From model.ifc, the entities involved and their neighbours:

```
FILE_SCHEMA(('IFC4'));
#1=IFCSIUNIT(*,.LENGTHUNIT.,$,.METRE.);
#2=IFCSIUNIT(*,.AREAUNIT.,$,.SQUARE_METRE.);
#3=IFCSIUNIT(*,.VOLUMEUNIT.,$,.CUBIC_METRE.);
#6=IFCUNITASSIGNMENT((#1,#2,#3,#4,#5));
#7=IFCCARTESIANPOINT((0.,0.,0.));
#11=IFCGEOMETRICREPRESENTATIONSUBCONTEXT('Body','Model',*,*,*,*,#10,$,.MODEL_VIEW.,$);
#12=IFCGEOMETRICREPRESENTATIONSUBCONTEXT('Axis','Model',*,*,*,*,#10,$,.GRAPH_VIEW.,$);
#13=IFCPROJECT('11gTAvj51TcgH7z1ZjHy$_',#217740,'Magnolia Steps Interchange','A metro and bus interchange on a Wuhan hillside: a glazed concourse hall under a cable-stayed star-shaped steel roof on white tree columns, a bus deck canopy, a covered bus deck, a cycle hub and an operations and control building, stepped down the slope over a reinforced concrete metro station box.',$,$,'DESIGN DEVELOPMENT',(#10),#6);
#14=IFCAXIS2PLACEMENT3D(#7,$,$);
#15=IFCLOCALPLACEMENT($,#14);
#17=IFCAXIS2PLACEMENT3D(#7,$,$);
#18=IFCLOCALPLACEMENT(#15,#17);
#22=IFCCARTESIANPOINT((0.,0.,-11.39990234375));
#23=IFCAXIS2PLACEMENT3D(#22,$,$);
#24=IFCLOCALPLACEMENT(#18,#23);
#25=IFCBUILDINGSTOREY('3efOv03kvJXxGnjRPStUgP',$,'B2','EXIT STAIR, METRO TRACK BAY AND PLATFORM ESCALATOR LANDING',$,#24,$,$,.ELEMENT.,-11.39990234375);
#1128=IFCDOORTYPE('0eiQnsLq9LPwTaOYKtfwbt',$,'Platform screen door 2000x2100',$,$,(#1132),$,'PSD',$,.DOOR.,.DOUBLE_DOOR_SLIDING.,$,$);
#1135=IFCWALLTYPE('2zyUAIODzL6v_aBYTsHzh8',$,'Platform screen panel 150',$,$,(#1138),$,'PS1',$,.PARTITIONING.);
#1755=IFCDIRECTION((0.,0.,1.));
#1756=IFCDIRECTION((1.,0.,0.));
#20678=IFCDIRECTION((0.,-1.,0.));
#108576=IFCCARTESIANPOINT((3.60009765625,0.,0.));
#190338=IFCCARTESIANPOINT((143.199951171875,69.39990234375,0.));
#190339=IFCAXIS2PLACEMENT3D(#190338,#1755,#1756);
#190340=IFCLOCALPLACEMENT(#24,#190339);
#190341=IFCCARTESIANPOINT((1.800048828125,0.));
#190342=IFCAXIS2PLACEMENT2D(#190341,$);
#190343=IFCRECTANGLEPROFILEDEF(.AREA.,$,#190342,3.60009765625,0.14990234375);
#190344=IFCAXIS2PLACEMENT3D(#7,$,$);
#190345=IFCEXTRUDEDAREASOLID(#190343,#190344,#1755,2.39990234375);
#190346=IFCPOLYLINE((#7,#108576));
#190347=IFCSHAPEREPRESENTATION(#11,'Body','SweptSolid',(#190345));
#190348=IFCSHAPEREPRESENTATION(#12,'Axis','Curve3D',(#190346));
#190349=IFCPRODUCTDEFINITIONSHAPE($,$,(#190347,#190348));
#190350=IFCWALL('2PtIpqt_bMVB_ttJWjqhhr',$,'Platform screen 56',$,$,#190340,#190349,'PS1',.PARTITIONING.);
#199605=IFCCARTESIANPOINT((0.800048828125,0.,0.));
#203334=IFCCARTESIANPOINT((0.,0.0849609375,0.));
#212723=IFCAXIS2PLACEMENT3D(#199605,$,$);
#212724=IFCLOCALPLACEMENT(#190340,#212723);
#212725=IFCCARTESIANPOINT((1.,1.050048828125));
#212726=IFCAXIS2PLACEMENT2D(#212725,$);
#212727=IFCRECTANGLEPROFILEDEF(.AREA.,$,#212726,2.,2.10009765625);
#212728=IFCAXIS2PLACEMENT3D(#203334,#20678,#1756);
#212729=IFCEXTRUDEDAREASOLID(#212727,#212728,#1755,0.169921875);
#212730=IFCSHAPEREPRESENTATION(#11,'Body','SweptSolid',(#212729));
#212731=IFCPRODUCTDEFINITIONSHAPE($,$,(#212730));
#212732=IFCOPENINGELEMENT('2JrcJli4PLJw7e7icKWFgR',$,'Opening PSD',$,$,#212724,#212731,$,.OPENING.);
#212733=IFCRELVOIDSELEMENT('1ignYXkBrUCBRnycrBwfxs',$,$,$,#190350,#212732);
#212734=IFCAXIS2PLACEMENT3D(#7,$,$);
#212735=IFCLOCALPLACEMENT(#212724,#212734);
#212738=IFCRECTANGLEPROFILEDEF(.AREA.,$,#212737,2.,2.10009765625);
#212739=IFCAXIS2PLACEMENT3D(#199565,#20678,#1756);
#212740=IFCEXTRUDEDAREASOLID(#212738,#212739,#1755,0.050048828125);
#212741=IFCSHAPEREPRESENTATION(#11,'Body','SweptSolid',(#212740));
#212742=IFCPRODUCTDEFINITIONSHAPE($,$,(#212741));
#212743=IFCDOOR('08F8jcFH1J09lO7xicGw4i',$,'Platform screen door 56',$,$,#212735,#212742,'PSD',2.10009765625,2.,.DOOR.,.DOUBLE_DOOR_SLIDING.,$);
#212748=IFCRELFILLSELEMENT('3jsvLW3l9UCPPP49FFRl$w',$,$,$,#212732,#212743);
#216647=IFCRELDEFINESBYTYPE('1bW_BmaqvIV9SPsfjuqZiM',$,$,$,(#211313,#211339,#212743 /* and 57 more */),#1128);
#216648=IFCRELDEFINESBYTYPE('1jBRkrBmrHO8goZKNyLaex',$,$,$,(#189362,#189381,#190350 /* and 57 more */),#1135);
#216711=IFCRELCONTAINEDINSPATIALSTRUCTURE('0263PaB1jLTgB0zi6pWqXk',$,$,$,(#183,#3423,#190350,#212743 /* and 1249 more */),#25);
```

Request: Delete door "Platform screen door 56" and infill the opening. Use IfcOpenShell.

```python
import ifcopenshell
import ifcopenshell.api.feature
import ifcopenshell.api.root
import ifcopenshell.geom
import ifcopenshell.util.shape

model = ifcopenshell.open("model.ifc")
settings = ifcopenshell.geom.settings()


def volume(element):
    """Net volume in cubic metres, openings subtracted."""
    shape = ifcopenshell.geom.create_shape(settings, element)
    return ifcopenshell.util.shape.get_volume(shape.geometry)


door = model.by_guid("08F8jcFH1J09lO7xicGw4i")
opening = door.FillsVoids[0].RelatingOpeningElement
wall = opening.VoidsElements[0].RelatingBuildingElement
before = volume(wall)

ifcopenshell.api.root.remove_product(model, product=door)
ifcopenshell.api.feature.remove_feature(model, feature=opening)

after = volume(wall)

print(f"wall volume {before:.3f} -> {after:.3f} m3")

model.write("model_edited.ifc")
```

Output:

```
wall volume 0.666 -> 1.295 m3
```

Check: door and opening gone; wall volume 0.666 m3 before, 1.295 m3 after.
